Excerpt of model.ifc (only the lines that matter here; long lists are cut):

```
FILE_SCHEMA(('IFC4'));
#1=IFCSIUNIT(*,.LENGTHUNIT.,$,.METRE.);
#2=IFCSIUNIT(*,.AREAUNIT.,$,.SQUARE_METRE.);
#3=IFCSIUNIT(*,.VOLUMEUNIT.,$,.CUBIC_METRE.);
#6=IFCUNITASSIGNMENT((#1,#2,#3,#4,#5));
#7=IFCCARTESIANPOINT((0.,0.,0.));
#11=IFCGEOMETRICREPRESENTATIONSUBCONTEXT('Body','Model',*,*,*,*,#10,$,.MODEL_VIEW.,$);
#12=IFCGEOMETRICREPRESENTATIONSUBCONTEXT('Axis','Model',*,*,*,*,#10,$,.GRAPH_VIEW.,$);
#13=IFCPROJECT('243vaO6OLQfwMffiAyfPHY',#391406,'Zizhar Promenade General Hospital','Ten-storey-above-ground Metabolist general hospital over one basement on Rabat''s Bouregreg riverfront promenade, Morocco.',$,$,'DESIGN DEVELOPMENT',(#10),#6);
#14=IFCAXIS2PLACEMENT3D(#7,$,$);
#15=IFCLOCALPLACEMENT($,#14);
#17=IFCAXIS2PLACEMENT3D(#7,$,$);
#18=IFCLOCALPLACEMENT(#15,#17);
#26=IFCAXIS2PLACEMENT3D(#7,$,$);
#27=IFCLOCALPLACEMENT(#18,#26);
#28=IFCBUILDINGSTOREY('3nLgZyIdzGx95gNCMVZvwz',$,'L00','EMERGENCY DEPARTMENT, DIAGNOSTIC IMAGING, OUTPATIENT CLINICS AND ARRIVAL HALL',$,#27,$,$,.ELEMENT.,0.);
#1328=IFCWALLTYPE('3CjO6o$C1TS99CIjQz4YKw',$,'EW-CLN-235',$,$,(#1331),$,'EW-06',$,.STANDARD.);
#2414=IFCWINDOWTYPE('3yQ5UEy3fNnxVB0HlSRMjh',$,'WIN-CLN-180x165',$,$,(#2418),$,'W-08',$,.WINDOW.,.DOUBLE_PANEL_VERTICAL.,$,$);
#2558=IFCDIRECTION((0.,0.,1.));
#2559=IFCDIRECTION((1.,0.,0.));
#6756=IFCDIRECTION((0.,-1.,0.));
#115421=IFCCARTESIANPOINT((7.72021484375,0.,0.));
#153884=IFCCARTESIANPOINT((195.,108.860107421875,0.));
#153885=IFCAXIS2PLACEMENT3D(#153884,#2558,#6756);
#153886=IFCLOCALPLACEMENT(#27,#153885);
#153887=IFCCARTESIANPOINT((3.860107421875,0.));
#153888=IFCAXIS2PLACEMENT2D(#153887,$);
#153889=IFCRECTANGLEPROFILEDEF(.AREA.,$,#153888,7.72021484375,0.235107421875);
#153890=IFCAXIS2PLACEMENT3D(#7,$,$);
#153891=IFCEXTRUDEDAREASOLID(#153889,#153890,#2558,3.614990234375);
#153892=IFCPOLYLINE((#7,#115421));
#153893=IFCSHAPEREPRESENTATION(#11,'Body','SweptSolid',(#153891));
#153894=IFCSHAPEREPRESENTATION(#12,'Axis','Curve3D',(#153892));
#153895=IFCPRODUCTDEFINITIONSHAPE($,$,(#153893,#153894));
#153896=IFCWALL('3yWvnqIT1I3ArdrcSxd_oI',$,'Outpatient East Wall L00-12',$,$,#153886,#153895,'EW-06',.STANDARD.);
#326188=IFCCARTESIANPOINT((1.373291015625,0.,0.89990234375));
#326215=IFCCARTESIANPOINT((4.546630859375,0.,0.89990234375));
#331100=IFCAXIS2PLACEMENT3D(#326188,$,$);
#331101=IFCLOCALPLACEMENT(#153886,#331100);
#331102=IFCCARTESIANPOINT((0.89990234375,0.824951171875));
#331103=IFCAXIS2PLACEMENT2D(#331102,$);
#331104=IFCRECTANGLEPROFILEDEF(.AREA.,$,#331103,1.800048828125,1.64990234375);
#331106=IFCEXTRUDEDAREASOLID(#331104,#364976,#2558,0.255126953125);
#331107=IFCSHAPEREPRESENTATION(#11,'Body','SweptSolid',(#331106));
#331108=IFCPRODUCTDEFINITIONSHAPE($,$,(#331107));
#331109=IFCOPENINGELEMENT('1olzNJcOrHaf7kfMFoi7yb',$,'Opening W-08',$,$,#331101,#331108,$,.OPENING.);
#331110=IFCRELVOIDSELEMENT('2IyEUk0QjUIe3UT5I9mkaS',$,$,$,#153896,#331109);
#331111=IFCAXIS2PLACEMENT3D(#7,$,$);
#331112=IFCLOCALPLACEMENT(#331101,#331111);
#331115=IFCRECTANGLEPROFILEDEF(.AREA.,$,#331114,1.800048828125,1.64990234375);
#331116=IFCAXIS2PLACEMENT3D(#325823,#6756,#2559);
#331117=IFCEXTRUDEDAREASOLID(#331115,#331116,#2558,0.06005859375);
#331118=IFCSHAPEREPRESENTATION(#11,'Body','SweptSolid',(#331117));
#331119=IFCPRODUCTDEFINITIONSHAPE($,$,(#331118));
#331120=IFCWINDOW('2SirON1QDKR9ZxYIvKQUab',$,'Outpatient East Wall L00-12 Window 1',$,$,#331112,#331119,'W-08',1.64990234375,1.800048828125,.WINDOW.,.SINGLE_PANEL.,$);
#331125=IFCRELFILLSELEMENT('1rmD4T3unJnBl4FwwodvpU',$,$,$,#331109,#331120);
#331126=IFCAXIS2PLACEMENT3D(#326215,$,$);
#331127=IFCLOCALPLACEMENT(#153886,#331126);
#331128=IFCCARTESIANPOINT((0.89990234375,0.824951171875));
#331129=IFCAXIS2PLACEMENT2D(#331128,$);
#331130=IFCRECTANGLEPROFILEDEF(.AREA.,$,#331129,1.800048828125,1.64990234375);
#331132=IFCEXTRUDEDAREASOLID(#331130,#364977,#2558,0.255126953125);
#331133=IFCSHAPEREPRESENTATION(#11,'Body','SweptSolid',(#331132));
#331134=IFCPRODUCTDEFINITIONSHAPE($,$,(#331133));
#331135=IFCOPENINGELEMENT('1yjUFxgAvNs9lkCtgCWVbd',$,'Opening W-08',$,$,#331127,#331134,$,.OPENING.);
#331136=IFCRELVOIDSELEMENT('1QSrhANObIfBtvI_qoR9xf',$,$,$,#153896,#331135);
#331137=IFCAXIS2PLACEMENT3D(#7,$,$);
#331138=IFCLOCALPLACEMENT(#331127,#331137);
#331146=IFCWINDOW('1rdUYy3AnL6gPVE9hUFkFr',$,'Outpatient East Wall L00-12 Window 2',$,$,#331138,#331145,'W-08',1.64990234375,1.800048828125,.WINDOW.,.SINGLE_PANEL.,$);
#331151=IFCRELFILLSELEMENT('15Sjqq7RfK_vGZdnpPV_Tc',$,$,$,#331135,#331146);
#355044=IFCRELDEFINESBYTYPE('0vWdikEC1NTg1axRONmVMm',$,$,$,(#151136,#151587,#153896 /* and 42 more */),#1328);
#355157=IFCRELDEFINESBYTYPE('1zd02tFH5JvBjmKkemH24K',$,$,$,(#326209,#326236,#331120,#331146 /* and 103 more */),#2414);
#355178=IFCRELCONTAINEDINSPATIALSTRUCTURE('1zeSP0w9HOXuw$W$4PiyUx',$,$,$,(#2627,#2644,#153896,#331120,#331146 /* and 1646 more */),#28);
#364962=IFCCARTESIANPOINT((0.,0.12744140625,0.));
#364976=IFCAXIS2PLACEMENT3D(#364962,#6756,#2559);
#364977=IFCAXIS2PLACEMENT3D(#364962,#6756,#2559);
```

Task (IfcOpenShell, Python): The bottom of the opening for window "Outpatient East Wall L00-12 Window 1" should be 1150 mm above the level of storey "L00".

```python
import numpy as np
import ifcopenshell
import ifcopenshell.api.geometry
import ifcopenshell.geom
import ifcopenshell.util.element
import ifcopenshell.util.placement
import ifcopenshell.util.shape
import ifcopenshell.util.unit

model = ifcopenshell.open("model.ifc")
unit_scale = ifcopenshell.util.unit.calculate_unit_scale(model)

window = model.by_guid("2SirON1QDKR9ZxYIvKQUab")
opening = window.FillsVoids[0].RelatingOpeningElement
storey = ifcopenshell.util.element.get_container(window, ifc_class="IfcBuildingStorey")
level = ifcopenshell.util.placement.get_local_placement(storey.ObjectPlacement)[2, 3]

# The opening's origin need not be at the sill, so measure its lowest point.
shape = ifcopenshell.geom.create_shape(ifcopenshell.geom.settings(), opening)
bottom = ifcopenshell.util.shape.get_shape_bottom_elevation(shape, shape.geometry) / unit_scale
dz = level + 1.15 - bottom

shift = np.array([0.0, 0.0, dz])
# The window is placed relative to its opening, so it follows when the opening moves.
matrix = ifcopenshell.util.placement.get_local_placement(opening.ObjectPlacement)
matrix[:3, 3] += shift
ifcopenshell.api.geometry.edit_object_placement(
    model, product=opening, matrix=matrix, is_si=False, should_transform_children=True
)

print(f"moved by {dz * unit_scale:+.3f} m")

model.write("model-out.ifc")
```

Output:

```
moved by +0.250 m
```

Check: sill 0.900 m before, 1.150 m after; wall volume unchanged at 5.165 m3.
